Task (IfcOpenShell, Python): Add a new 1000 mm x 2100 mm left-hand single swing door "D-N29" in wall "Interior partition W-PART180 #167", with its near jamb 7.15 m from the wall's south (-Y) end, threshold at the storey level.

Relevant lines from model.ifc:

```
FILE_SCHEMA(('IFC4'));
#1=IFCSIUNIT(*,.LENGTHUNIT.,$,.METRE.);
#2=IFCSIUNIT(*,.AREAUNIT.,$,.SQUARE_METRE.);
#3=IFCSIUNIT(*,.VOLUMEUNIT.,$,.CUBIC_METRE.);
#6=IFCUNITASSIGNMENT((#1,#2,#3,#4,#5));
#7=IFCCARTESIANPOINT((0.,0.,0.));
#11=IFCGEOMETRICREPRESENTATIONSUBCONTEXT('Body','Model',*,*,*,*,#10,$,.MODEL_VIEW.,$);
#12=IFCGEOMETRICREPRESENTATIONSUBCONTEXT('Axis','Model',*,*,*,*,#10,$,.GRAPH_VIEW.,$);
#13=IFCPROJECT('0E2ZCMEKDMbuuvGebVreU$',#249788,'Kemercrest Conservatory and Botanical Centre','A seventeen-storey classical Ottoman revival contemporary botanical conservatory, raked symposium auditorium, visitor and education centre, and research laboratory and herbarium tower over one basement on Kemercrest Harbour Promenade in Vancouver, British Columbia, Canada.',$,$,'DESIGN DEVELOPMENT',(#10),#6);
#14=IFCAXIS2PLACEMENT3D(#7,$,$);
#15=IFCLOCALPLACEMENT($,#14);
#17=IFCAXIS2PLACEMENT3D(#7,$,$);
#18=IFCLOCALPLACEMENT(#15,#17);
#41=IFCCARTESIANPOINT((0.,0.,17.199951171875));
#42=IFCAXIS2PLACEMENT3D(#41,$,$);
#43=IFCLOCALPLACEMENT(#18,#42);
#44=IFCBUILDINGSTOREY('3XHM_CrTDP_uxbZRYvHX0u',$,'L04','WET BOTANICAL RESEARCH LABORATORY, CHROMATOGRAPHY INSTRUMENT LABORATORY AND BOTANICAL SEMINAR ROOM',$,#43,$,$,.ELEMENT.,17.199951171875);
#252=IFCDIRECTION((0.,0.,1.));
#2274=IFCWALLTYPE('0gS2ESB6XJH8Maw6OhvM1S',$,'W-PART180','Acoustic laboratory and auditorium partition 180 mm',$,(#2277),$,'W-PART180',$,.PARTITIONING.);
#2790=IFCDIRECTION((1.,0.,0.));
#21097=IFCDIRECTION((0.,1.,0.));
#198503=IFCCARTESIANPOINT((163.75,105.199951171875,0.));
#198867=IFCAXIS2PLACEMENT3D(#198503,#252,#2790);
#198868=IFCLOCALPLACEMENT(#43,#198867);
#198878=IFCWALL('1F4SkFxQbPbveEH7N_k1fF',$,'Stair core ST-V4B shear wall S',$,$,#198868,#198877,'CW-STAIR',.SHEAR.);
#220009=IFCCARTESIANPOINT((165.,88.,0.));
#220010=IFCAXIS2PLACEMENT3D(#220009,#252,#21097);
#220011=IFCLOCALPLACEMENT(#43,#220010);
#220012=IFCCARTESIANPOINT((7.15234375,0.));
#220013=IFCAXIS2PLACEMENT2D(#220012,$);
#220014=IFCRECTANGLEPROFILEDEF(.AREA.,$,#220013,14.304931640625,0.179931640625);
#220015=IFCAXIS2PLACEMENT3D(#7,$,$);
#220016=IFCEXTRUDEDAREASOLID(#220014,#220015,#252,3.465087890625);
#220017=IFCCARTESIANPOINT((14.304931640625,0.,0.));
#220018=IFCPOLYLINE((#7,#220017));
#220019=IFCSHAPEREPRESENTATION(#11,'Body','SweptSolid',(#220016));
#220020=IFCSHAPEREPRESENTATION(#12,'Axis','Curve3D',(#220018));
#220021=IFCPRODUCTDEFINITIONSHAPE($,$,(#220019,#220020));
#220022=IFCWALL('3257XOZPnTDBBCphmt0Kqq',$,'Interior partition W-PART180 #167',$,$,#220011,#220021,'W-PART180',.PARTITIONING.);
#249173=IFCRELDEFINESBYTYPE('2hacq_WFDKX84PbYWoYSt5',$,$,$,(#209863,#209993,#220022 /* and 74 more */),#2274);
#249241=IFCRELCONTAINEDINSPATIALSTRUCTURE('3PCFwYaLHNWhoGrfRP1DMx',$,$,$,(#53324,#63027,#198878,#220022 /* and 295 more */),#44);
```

```python
import numpy as np
import ifcopenshell
import ifcopenshell.api.feature
import ifcopenshell.api.geometry
import ifcopenshell.api.root
import ifcopenshell.api.spatial
import ifcopenshell.geom
import ifcopenshell.util.element
import ifcopenshell.util.placement
import ifcopenshell.util.representation
import ifcopenshell.util.shape
import ifcopenshell.util.unit

model = ifcopenshell.open("model.ifc")
unit_scale = ifcopenshell.util.unit.calculate_unit_scale(model)
settings = ifcopenshell.geom.settings()


def volume(element):
    """Net volume in cubic metres, openings subtracted."""
    shape = ifcopenshell.geom.create_shape(settings, element)
    return ifcopenshell.util.shape.get_volume(shape.geometry)


wall = model.by_guid("3257XOZPnTDBBCphmt0Kqq")
storey = ifcopenshell.util.element.get_container(wall, ifc_class="IfcBuildingStorey")
context = ifcopenshell.util.representation.get_context(model, "Model", "Body", "MODEL_VIEW")
before = volume(wall)

width, height, from_end, sill = 1, 2.1, 7.15, 0.0  # metres

# The wall runs along its own X axis, and the end named is its -X end.
wall_shape = ifcopenshell.geom.create_shape(settings, wall)
x, y, z = ifcopenshell.util.shape.get_vertices(wall_shape.geometry).T
start = x.min() + from_end
face, thickness = float(y.min()), float(y.max() - y.min())
wall_matrix = ifcopenshell.util.placement.get_local_placement(wall.ObjectPlacement)
level = ifcopenshell.util.placement.get_local_placement(storey.ObjectPlacement)[2, 3]


def in_wall(x, y):
    """Placement at x, y metres in the wall's axes, at sill height."""
    matrix = wall_matrix.copy()
    matrix[:, 3] = wall_matrix @ np.array([x / unit_scale, y / unit_scale, 0.0, 1.0])
    matrix[2, 3] = level + sill / unit_scale
    return matrix


# Opening: a box that overshoots both wall faces by 50 mm.
opening = ifcopenshell.api.root.create_entity(model, ifc_class="IfcOpeningElement", predefined_type="OPENING")
box = ifcopenshell.api.geometry.add_wall_representation(
    model, context=context, length=width, height=height, thickness=thickness + 0.1
)
ifcopenshell.api.geometry.assign_representation(model, product=opening, representation=box)
ifcopenshell.api.geometry.edit_object_placement(model, product=opening, matrix=in_wall(start, face - 0.05), is_si=False)
ifcopenshell.api.feature.add_feature(model, feature=opening, element=wall)

door = ifcopenshell.api.root.create_entity(model, ifc_class="IfcDoor", name="D-N29", predefined_type="DOOR")
door.OverallWidth, door.OverallHeight = width / unit_scale, height / unit_scale
door.OperationType = "SINGLE_SWING_LEFT"
body = ifcopenshell.api.geometry.add_door_representation(
    model,
    context=context,
    overall_width=door.OverallWidth,
    overall_height=door.OverallHeight,
    operation_type="SINGLE_SWING_LEFT",
    lining_properties={"LiningDepth": thickness / unit_scale, "ThresholdDepth": thickness / unit_scale},
)
ifcopenshell.api.geometry.assign_representation(model, product=door, representation=body)
ifcopenshell.api.spatial.assign_container(model, products=[door], relating_structure=storey)
ifcopenshell.api.feature.add_filling(model, opening=opening, element=door)

# The lining spans the wall, so the door starts at the wall face.
ifcopenshell.api.geometry.edit_object_placement(model, product=door, matrix=in_wall(start, face), is_si=False)

after = volume(wall)

print(f"wall volume {before:.3f} -> {after:.3f} m3")

model.write("model_v2.ifc")
```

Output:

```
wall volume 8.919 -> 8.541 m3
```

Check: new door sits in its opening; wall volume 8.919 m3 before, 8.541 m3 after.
